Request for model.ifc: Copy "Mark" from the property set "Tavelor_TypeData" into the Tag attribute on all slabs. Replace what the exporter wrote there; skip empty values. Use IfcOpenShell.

First a look at what the model holds.

```python
import ifcopenshell
import ifcopenshell.util.element

model = ifcopenshell.open("model.ifc")
print(model.schema)
slabs = model.by_type("IfcSlab")
print(len(slabs), "slabs")
for e in slabs[:8]:
    source = ifcopenshell.util.element.get_pset(e, "Tavelor_TypeData", "Mark")
    target = e.Tag
    print(e.id(), repr(source), repr(target), sep=" | ")
```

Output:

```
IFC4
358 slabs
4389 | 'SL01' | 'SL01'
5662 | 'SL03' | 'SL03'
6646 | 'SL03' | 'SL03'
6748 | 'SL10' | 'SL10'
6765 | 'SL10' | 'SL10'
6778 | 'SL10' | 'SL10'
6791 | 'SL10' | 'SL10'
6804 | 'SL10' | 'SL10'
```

```python
import ifcopenshell
import ifcopenshell.util.element

model = ifcopenshell.open("model.ifc")

count = 0
for e in model.by_type("IfcSlab"):
    value = ifcopenshell.util.element.get_pset(e, "Tavelor_TypeData", "Mark")
    current = e.Tag
    if not value or not value.strip() or current == value:
        continue
    e.Tag = value
    count += 1

print(count, "slabs updated")

model.write("model-out.ifc")
```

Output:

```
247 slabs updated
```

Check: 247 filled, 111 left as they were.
